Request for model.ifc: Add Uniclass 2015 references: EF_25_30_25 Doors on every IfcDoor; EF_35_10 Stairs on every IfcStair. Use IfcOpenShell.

First a look at what the model holds.

```python
import ifcopenshell

model = ifcopenshell.open("model.ifc")
print(model.schema)
print("classifications:", [c.Name for c in model.by_type("IfcClassification")])
for ifc_class in ("IfcDoor", "IfcRoof", "IfcStair", "IfcWall", "IfcWindow"):
    print(ifc_class, len(model.by_type(ifc_class)))
```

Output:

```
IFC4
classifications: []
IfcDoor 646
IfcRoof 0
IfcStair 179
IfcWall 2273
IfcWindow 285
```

```python
import ifcopenshell
import ifcopenshell.api.classification

model = ifcopenshell.open("model.ifc")

system = ifcopenshell.api.classification.add_classification(model, classification="Uniclass 2015")

codes = {
    "IfcDoor": ("EF_25_30_25", "Doors"),
    "IfcStair": ("EF_35_10", "Stairs"),
}
for ifc_class, (code, name) in codes.items():
    products = model.by_type(ifc_class)
    ifcopenshell.api.classification.add_reference(
        model, products=products, classification=system, identification=code, name=name
    )
    print(code, len(products))

model.write("model_rev.ifc")
```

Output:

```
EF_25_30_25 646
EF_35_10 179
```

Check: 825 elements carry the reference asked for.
